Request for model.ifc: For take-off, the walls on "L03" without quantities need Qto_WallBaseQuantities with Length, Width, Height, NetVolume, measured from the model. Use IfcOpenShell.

First a look at what the model holds.

```python
import ifcopenshell
import ifcopenshell.util.element
import ifcopenshell.util.unit

model = ifcopenshell.open("model.ifc")
print(model.schema)
for unit_type in ("LENGTHUNIT", "AREAUNIT", "VOLUMEUNIT"):
    print(unit_type, ifcopenshell.util.unit.calculate_unit_scale(model, unit_type))
storey = next(s for s in model.by_type("IfcBuildingStorey") if s.Name == "L03")
walls = [e for e in ifcopenshell.util.element.get_decomposition(storey) if e.is_a("IfcWall")]
for e in sorted(walls, key=lambda e: e.id()):
    print(e.id(), e.is_a(), e.Name, list(ifcopenshell.util.element.get_psets(e, qtos_only=True)), sep=" | ")
```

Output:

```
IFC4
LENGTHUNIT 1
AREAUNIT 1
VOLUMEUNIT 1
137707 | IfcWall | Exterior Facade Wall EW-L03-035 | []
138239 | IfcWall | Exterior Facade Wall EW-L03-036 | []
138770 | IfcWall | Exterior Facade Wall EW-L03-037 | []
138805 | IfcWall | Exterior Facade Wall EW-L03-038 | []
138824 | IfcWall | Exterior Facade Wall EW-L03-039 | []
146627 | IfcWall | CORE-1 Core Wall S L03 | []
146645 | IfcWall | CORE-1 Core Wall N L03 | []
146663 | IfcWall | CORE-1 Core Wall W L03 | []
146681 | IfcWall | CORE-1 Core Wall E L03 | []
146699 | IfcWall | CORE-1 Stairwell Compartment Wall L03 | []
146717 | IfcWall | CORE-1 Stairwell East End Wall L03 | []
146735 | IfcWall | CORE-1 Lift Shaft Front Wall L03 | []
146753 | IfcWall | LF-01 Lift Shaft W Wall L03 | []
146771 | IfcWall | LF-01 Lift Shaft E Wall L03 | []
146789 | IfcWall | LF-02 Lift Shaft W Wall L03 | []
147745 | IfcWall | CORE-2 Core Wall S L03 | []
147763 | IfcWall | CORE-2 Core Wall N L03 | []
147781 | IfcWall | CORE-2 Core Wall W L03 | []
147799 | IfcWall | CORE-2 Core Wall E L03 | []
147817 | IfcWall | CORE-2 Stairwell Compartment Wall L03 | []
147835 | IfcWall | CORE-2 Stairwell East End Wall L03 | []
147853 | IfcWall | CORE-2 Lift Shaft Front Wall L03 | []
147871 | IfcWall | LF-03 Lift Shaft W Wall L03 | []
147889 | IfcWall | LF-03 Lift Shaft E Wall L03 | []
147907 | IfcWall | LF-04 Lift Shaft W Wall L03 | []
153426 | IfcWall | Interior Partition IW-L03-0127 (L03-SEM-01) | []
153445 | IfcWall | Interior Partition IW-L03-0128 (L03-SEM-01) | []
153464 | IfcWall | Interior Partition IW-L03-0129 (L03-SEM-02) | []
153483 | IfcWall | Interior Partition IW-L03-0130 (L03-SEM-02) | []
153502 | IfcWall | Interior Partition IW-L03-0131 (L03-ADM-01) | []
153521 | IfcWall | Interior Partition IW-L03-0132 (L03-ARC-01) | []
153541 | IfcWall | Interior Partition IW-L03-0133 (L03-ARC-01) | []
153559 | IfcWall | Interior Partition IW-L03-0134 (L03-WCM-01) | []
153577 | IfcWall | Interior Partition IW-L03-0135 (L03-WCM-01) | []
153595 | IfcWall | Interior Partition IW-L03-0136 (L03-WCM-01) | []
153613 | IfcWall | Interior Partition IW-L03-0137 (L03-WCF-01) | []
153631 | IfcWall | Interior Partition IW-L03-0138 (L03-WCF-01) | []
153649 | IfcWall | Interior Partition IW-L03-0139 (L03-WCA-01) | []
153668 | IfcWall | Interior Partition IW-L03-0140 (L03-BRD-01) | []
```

```python
import ifcopenshell
import ifcopenshell.api.pset
import ifcopenshell.geom
import ifcopenshell.util.element
import ifcopenshell.util.shape
import ifcopenshell.util.unit

model = ifcopenshell.open("model.ifc")
unit_scale = ifcopenshell.util.unit.calculate_unit_scale(model)
volume_scale = ifcopenshell.util.unit.calculate_unit_scale(model, "VOLUMEUNIT")
settings = ifcopenshell.geom.settings()

storey = next(s for s in model.by_type("IfcBuildingStorey") if s.Name == "L03")
walls = [e for e in ifcopenshell.util.element.get_decomposition(storey) if e.is_a("IfcWall")]

for e in sorted(walls, key=lambda e: e.id()):
    if ifcopenshell.util.element.get_psets(e, qtos_only=True, should_inherit=False):
        continue
    # Geometry comes back in metres, in the element's own axes.
    shape = ifcopenshell.geom.create_shape(settings, e)
    values = {
        "Length": ifcopenshell.util.shape.get_x(shape.geometry) / unit_scale,
        "Width": ifcopenshell.util.shape.get_y(shape.geometry) / unit_scale,
        "Height": ifcopenshell.util.shape.get_z(shape.geometry) / unit_scale,
        "NetVolume": ifcopenshell.util.shape.get_volume(shape.geometry) / volume_scale,
    }
    qto = ifcopenshell.api.pset.add_qto(model, product=e, name="Qto_WallBaseQuantities")
    ifcopenshell.api.pset.edit_qto(model, qto=qto, properties=values)
    print(e.id(), {k: round(v, 3) for k, v in values.items()})

model.write("model_edited.ifc")
```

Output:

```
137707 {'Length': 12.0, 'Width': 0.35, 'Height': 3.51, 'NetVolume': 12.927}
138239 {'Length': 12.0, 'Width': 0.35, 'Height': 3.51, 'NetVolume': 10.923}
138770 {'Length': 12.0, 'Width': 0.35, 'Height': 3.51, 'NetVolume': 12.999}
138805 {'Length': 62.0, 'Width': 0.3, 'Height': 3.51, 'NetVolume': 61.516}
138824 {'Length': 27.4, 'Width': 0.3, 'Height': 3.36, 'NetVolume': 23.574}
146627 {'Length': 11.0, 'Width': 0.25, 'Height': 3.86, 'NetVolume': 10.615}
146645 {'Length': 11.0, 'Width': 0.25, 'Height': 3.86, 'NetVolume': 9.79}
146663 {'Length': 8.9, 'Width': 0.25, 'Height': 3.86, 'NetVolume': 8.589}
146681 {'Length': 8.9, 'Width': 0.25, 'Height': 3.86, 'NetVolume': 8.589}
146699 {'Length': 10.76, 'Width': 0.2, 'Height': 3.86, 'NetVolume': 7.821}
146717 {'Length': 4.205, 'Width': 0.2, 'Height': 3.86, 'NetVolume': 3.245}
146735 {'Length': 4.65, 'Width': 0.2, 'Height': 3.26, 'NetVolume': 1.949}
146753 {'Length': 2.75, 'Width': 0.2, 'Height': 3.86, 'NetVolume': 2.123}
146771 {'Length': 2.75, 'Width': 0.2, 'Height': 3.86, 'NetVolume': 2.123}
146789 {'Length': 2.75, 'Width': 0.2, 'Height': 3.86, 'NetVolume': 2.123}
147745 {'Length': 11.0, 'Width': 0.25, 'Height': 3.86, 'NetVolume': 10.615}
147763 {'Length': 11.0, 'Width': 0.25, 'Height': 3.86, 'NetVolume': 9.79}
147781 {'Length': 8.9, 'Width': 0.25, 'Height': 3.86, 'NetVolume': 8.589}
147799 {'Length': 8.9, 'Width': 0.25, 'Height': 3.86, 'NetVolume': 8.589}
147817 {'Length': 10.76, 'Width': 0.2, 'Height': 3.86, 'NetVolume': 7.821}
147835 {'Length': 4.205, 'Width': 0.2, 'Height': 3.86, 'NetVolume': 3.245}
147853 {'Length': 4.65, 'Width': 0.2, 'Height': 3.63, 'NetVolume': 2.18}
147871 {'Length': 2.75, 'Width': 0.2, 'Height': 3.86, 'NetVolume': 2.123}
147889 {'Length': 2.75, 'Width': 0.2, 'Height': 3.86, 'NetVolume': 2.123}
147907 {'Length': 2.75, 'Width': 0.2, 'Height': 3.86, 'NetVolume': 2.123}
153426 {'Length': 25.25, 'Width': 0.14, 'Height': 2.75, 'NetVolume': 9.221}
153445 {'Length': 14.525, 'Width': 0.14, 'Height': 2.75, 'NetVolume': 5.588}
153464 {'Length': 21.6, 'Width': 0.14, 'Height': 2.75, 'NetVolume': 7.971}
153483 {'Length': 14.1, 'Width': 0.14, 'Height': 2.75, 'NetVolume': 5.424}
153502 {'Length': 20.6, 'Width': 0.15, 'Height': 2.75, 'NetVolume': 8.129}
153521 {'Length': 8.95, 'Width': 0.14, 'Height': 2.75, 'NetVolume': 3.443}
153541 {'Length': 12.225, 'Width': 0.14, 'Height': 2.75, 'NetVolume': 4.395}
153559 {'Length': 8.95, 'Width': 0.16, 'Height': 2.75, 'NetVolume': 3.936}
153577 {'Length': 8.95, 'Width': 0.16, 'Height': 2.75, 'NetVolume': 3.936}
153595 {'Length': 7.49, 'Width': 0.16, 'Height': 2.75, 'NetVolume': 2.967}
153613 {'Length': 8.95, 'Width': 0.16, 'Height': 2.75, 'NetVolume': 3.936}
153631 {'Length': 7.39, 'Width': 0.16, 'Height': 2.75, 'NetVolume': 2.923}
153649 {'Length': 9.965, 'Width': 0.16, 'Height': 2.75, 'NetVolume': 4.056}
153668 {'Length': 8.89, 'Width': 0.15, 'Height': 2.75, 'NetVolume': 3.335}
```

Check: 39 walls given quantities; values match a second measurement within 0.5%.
